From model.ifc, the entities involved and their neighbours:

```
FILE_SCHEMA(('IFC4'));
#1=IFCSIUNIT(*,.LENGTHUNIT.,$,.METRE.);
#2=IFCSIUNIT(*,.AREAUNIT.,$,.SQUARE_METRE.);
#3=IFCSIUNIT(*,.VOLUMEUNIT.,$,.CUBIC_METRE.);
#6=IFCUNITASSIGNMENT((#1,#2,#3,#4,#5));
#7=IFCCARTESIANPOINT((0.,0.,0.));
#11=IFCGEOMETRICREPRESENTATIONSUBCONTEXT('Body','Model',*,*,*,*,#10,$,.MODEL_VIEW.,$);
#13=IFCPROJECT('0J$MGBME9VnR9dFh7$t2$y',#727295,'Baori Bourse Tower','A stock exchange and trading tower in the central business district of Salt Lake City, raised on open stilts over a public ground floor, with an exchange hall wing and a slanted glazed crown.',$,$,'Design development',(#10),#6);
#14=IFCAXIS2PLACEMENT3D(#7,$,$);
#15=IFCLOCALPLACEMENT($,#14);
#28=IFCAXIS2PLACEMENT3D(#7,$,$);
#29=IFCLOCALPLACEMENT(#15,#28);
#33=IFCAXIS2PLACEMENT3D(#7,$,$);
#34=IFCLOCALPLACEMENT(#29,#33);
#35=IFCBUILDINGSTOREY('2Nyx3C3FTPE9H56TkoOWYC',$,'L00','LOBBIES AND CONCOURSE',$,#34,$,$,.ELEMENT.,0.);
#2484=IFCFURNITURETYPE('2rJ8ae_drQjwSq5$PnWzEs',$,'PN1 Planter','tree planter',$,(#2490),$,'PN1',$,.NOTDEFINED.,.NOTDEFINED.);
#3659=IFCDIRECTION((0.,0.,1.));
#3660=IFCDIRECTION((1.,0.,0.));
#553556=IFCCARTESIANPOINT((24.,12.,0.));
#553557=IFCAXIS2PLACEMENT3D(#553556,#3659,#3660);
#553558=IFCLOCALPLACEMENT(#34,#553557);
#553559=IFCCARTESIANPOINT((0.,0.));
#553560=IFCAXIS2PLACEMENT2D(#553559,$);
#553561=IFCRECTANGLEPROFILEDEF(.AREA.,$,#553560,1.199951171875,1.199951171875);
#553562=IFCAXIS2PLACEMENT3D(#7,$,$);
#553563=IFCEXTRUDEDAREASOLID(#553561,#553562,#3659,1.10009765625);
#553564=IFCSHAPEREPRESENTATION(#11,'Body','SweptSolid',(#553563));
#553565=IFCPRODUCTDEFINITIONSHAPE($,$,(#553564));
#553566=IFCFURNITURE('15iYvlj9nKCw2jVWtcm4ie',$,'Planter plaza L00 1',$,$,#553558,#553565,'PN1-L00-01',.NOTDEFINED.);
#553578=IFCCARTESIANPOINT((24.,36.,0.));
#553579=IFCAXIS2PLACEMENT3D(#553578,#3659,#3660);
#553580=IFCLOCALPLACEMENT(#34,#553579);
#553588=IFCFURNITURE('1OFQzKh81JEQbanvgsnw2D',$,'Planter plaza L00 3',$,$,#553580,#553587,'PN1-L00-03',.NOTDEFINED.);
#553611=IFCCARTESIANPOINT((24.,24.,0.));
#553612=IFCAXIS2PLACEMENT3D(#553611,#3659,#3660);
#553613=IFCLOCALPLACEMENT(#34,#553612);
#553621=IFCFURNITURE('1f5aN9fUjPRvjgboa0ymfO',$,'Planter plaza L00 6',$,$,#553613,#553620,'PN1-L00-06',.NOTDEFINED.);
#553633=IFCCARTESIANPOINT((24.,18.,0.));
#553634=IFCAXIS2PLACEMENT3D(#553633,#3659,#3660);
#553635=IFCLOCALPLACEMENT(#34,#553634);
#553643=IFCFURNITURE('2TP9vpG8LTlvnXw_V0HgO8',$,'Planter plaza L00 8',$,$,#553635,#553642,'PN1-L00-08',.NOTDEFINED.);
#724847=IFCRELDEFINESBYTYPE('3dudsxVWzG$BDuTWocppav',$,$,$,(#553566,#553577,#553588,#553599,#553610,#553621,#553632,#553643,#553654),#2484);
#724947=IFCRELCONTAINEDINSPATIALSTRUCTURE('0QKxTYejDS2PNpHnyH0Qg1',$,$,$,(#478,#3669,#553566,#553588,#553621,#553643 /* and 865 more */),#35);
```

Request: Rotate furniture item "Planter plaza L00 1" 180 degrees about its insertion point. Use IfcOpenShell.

```python
import ifcopenshell
import ifcopenshell.api.geometry
import ifcopenshell.util.placement

model = ifcopenshell.open("model.ifc")

item = model.by_guid("15iYvlj9nKCw2jVWtcm4ie")
matrix = ifcopenshell.util.placement.get_local_placement(item.ObjectPlacement)
matrix = matrix @ ifcopenshell.util.placement.rotation(180, "Z")
ifcopenshell.api.geometry.edit_object_placement(model, product=item, matrix=matrix, is_si=False)

print(ifcopenshell.util.placement.get_local_placement(item.ObjectPlacement).round(3) + 0.0)

model.write("model_updated.ifc")
```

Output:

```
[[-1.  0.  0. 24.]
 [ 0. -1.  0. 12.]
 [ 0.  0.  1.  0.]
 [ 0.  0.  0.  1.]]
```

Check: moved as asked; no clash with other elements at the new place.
